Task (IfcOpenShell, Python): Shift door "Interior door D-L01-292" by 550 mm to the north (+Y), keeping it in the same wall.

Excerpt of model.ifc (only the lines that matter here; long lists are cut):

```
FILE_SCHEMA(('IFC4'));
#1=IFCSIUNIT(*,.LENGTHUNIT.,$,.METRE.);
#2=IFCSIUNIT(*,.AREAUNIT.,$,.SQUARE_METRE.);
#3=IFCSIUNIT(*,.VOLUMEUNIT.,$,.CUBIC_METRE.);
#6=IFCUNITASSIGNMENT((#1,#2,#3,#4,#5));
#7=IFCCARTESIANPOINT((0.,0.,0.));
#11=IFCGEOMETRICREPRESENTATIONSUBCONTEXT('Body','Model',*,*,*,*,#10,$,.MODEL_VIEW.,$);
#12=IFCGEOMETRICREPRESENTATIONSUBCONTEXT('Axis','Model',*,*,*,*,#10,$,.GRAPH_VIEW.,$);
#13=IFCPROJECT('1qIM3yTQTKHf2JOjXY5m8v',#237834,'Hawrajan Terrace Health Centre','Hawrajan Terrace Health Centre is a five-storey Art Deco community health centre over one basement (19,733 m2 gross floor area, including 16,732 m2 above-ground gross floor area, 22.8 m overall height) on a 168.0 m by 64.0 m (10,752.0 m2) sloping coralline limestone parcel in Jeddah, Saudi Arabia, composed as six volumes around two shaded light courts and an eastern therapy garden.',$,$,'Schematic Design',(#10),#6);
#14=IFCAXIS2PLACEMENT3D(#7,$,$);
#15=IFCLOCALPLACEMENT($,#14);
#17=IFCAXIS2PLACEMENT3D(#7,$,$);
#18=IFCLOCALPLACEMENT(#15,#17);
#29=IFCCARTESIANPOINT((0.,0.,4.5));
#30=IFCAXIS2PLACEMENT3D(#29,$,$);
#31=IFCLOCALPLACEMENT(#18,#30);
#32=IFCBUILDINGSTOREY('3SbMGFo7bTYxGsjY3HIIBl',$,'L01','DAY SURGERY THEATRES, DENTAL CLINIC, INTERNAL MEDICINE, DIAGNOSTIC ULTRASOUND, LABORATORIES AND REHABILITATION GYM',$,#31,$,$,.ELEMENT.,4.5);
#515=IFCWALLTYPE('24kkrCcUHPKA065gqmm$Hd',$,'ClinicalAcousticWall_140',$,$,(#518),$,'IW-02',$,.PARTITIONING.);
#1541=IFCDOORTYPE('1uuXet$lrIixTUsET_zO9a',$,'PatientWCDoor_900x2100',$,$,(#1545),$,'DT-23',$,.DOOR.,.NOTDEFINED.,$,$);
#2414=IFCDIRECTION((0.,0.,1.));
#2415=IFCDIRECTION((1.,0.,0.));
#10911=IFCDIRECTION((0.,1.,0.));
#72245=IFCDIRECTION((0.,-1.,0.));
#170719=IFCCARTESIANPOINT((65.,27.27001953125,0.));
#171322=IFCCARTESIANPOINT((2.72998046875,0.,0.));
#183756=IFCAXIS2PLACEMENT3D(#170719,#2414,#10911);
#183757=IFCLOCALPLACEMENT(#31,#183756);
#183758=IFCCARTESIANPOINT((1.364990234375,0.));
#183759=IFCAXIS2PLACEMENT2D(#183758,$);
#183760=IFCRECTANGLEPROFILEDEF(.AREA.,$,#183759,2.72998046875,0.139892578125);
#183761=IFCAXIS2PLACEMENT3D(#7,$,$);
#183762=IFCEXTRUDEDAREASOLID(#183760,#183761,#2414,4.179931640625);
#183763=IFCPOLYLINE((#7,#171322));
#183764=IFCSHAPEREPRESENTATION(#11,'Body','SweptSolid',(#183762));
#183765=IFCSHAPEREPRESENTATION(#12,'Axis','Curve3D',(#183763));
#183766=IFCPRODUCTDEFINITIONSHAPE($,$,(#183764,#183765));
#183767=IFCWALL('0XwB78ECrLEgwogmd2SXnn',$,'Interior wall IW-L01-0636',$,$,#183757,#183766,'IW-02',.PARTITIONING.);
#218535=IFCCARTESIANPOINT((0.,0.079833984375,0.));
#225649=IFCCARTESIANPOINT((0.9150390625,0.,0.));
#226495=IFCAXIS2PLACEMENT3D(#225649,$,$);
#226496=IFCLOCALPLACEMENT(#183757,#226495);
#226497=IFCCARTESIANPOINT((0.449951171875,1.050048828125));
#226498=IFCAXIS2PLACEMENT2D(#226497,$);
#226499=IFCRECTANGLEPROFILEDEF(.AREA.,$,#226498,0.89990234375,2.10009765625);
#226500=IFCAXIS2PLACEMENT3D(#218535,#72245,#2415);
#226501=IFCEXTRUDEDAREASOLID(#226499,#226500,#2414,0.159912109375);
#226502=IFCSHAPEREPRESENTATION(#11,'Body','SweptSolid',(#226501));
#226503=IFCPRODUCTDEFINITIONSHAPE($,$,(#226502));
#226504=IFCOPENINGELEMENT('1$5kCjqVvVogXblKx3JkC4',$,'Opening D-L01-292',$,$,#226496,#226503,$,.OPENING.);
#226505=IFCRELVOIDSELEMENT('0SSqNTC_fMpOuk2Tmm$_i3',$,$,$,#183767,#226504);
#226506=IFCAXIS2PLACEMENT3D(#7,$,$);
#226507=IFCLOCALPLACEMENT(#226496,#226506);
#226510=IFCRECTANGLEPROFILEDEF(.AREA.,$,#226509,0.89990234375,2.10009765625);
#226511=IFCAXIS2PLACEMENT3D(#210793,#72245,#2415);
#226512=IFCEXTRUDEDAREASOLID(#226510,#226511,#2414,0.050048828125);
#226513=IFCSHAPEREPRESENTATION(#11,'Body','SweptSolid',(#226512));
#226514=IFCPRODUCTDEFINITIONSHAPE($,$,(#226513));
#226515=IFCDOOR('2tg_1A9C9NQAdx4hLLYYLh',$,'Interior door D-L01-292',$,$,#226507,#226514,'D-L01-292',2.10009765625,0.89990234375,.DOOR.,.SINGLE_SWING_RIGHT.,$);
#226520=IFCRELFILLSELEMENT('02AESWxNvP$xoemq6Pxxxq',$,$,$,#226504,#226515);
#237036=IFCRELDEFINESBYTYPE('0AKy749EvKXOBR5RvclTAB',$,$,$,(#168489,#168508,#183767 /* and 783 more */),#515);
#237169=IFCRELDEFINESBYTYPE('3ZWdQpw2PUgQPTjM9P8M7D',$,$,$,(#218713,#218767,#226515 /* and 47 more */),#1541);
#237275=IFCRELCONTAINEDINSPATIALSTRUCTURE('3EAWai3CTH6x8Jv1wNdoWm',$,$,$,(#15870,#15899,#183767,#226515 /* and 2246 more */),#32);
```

```python
import ifcopenshell
import ifcopenshell.api.geometry
import ifcopenshell.util.placement
import ifcopenshell.util.unit

model = ifcopenshell.open("model.ifc")
unit_scale = ifcopenshell.util.unit.calculate_unit_scale(model)

door = model.by_guid("2tg_1A9C9NQAdx4hLLYYLh")
opening = door.FillsVoids[0].RelatingOpeningElement
wall = opening.VoidsElements[0].RelatingBuildingElement

wall_matrix = ifcopenshell.util.placement.get_local_placement(wall.ObjectPlacement)
shift = wall_matrix[:3, 0] * 0.55 / unit_scale
before = ifcopenshell.util.placement.get_local_placement(door.ObjectPlacement)[:3, 3].copy()

# The door is placed relative to its opening, so it follows when the opening moves.
matrix = ifcopenshell.util.placement.get_local_placement(opening.ObjectPlacement)
matrix[:3, 3] += shift
ifcopenshell.api.geometry.edit_object_placement(
    model, product=opening, matrix=matrix, is_si=False, should_transform_children=True
)

after = ifcopenshell.util.placement.get_local_placement(door.ObjectPlacement)[:3, 3]
print("door moved by", (after - before).round(3) + 0.0)

model.write("model_updated.ifc")
```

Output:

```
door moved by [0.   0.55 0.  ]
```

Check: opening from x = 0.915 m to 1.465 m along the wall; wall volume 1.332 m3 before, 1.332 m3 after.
